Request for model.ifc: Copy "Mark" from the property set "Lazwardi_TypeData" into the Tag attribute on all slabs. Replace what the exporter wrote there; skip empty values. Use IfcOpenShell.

First a look at what the model holds.

```python
import ifcopenshell
import ifcopenshell.util.element

model = ifcopenshell.open("model.ifc")
print(model.schema)
slabs = model.by_type("IfcSlab")
print(len(slabs), "slabs")
for e in slabs[:8]:
    source = ifcopenshell.util.element.get_pset(e, "Lazwardi_TypeData", "Mark")
    target = e.Tag
    print(e.id(), repr(source), repr(target), sep=" | ")
```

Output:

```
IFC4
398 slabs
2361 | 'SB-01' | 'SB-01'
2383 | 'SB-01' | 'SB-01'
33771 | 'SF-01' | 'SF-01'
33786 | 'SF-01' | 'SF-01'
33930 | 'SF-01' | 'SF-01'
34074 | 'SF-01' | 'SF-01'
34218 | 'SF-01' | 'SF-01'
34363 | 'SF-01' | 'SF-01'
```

```python
import ifcopenshell
import ifcopenshell.util.element

model = ifcopenshell.open("model.ifc")

count = 0
for e in model.by_type("IfcSlab"):
    value = ifcopenshell.util.element.get_pset(e, "Lazwardi_TypeData", "Mark")
    current = e.Tag
    if not value or not value.strip() or current == value:
        continue
    e.Tag = value
    count += 1

print(count, "slabs updated")

model.write("model-out.ifc")
```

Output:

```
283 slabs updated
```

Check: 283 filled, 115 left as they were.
